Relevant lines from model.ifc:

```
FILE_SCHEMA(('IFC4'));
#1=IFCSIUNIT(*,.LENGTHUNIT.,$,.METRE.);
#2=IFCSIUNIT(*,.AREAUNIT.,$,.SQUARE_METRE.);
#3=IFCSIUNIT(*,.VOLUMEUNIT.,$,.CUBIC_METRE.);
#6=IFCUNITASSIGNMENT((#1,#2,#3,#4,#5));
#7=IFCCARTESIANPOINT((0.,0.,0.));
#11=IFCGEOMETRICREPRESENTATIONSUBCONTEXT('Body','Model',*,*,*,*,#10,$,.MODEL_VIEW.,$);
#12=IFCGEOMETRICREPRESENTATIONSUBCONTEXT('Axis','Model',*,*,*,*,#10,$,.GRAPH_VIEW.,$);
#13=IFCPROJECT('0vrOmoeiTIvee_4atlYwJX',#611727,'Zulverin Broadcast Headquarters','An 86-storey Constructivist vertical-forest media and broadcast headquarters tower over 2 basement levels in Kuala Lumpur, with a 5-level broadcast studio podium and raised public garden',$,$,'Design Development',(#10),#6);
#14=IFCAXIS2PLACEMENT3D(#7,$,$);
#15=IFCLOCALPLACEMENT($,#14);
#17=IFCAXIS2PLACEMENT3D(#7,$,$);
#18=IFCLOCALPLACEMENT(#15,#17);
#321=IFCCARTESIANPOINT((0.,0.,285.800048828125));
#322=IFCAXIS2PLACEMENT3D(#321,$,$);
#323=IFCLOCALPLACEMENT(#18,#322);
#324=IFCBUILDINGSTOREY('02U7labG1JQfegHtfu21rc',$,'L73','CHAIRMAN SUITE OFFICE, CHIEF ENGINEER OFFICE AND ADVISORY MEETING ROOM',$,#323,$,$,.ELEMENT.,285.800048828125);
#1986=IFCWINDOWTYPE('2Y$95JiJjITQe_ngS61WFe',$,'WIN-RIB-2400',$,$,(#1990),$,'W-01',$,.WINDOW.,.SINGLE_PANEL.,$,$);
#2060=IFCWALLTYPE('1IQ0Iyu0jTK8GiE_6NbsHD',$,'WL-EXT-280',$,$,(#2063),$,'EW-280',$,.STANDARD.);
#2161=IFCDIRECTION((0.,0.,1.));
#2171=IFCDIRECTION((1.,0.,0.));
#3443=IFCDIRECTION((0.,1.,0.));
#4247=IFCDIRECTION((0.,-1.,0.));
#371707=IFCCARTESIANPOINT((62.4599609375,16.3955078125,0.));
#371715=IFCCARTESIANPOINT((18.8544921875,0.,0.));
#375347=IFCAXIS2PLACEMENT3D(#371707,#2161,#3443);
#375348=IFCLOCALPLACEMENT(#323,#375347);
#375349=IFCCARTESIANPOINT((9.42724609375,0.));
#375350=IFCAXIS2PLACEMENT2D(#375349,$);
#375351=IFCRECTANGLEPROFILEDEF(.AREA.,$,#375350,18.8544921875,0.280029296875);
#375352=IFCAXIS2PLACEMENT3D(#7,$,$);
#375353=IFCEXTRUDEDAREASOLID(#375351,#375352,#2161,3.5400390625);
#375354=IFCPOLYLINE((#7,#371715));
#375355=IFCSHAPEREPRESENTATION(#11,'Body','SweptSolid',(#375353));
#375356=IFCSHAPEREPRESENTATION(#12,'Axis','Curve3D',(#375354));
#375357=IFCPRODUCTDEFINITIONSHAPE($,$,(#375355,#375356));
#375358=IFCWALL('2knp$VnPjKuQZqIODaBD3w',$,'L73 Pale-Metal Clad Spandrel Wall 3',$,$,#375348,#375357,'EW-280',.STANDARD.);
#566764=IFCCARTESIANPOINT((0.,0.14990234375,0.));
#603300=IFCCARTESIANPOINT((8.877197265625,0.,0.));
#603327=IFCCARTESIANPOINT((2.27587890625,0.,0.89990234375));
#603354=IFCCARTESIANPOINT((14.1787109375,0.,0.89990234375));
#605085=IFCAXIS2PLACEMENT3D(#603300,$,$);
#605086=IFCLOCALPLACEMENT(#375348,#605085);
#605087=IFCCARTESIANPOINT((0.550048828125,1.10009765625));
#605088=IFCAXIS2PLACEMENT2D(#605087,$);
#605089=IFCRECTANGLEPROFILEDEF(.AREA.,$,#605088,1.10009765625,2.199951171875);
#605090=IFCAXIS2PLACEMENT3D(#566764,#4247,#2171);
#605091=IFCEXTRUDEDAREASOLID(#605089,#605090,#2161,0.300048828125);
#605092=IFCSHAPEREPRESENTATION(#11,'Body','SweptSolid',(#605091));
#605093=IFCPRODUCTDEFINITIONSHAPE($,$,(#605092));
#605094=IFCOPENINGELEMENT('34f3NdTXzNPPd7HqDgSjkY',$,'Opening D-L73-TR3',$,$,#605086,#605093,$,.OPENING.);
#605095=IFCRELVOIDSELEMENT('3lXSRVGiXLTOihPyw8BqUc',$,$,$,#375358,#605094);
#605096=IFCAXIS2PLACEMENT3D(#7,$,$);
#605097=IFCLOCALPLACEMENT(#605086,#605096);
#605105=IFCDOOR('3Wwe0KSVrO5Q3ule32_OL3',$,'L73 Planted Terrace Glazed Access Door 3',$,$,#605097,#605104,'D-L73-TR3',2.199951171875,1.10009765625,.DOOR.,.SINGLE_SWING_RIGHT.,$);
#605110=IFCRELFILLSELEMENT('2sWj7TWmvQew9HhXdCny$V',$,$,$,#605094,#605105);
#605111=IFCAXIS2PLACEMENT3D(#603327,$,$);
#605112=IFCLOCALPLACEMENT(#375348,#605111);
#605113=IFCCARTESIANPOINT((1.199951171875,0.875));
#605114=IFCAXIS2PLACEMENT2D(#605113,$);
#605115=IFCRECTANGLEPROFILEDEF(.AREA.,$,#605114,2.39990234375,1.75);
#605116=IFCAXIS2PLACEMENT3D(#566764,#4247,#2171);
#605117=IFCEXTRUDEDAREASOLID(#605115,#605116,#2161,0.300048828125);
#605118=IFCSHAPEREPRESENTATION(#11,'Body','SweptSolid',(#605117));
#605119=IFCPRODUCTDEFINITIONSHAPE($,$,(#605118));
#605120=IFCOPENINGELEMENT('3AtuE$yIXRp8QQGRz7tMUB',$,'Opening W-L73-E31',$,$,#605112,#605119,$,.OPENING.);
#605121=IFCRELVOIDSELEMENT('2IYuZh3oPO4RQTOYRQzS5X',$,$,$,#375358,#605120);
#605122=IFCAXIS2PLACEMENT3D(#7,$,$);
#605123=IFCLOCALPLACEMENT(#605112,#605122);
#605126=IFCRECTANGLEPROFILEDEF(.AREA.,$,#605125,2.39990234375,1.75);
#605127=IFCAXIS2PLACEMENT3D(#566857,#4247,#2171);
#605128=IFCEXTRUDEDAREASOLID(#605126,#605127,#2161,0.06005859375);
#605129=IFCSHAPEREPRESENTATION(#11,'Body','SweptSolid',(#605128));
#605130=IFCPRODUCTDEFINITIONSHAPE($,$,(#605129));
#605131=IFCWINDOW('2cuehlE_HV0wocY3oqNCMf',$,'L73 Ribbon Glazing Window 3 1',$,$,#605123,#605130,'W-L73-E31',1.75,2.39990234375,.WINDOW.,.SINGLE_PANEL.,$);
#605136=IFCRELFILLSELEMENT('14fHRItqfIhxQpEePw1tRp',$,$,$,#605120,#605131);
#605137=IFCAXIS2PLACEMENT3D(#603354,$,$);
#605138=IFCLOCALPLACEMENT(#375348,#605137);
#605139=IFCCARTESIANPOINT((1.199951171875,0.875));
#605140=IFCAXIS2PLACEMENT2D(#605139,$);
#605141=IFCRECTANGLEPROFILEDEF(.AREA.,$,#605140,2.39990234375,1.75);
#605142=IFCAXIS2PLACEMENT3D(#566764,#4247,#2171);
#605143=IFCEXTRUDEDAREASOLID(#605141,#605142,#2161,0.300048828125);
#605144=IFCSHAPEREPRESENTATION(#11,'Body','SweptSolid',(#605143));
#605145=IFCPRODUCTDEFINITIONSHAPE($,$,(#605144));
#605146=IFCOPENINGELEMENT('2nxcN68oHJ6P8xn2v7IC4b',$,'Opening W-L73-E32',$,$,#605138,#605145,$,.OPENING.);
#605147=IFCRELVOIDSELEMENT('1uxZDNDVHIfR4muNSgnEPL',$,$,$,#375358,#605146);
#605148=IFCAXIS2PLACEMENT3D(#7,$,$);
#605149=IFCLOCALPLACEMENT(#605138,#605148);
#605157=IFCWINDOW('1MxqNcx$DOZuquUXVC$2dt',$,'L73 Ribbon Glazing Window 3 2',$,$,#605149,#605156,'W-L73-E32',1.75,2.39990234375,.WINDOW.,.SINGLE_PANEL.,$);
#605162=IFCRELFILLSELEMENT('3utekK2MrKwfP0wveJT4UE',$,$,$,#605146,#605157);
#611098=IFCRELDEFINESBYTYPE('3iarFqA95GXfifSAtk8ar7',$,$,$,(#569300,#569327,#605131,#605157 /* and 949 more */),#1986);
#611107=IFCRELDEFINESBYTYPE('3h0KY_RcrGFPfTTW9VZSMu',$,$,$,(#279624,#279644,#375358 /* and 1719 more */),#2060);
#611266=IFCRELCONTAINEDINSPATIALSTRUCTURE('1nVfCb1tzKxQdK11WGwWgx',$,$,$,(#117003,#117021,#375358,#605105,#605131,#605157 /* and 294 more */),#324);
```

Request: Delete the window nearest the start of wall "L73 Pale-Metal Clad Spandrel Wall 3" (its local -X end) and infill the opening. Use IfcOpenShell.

```python
import ifcopenshell
import ifcopenshell.api.feature
import ifcopenshell.api.root
import ifcopenshell.geom
import ifcopenshell.util.shape

model = ifcopenshell.open("model.ifc")
settings = ifcopenshell.geom.settings()


def volume(element):
    """Net volume in cubic metres, openings subtracted."""
    shape = ifcopenshell.geom.create_shape(settings, element)
    return ifcopenshell.util.shape.get_volume(shape.geometry)


window = model.by_id(605131)
opening = window.FillsVoids[0].RelatingOpeningElement
wall = opening.VoidsElements[0].RelatingBuildingElement
before = volume(wall)

ifcopenshell.api.root.remove_product(model, product=window)
ifcopenshell.api.feature.remove_feature(model, feature=opening)

after = volume(wall)

print(f"wall volume {before:.3f} -> {after:.3f} m3")

model.write("model_edited.ifc")
```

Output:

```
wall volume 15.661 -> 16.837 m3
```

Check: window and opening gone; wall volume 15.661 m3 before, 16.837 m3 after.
